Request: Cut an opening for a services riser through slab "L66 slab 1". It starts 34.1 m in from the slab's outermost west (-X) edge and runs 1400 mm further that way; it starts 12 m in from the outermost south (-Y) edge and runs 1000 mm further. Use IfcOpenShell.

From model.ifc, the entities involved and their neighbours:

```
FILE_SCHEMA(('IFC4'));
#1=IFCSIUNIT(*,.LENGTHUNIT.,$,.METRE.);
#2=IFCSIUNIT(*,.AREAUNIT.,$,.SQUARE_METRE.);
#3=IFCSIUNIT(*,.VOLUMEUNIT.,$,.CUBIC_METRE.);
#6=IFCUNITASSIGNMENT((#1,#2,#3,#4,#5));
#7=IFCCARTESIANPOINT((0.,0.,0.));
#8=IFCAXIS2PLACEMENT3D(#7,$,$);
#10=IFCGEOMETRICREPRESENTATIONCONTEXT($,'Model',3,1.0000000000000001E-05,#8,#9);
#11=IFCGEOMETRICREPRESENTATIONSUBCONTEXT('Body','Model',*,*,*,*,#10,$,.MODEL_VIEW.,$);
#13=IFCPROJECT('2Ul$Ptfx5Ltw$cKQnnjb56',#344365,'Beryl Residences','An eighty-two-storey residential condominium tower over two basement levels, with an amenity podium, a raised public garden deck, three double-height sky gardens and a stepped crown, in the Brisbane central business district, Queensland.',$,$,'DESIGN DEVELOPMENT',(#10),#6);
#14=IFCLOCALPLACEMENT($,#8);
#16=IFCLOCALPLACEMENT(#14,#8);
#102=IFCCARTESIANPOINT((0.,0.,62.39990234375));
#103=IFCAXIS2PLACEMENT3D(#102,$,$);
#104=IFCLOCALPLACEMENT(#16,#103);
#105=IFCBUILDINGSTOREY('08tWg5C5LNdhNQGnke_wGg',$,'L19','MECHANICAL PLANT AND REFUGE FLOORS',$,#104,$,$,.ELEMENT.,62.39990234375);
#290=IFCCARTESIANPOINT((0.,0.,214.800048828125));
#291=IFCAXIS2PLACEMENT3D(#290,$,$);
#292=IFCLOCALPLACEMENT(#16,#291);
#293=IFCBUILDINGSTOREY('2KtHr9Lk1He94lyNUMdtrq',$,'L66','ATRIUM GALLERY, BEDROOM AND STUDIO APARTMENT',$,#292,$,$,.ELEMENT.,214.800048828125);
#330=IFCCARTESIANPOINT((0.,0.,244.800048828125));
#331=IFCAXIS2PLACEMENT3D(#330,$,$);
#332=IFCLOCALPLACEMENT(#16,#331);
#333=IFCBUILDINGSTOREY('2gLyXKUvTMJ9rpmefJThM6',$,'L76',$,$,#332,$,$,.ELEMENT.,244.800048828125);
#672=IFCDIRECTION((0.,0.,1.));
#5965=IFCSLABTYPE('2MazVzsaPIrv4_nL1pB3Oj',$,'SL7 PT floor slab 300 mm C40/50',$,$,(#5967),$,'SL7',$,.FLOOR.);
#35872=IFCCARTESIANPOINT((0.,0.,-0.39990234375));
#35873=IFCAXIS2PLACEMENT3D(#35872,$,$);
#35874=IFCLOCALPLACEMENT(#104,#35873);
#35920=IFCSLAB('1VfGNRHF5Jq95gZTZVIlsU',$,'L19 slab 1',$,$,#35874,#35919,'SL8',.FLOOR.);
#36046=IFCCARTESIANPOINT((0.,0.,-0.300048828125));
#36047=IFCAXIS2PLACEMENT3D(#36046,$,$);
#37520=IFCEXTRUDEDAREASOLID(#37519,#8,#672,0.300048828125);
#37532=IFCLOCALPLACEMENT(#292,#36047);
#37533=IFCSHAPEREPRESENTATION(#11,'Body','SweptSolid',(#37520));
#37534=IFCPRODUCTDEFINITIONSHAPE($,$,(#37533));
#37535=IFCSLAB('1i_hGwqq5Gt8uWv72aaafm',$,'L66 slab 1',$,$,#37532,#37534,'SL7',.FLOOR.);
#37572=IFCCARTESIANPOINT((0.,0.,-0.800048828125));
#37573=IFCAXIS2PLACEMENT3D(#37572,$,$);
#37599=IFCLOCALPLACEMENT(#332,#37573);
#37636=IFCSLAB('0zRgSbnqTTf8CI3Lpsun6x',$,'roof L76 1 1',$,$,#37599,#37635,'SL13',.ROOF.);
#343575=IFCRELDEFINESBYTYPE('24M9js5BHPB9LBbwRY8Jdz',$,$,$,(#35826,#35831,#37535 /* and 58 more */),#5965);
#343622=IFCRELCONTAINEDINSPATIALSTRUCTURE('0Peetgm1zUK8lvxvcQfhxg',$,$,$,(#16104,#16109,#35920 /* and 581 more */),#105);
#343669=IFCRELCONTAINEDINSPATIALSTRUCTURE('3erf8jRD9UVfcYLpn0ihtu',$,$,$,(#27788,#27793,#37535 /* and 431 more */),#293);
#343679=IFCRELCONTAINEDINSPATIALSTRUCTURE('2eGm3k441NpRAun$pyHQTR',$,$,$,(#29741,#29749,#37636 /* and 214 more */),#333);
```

```python
import numpy as np
import ifcopenshell
import ifcopenshell.api.feature
import ifcopenshell.api.geometry
import ifcopenshell.api.root
import ifcopenshell.geom
import ifcopenshell.util.placement
import ifcopenshell.util.representation
import ifcopenshell.util.shape
import ifcopenshell.util.unit

model = ifcopenshell.open("model.ifc")
unit_scale = ifcopenshell.util.unit.calculate_unit_scale(model)
settings = ifcopenshell.geom.settings()


def volume(element):
    """Net volume in cubic metres, openings subtracted."""
    shape = ifcopenshell.geom.create_shape(settings, element)
    return ifcopenshell.util.shape.get_volume(shape.geometry)


slab = model.by_guid("1i_hGwqq5Gt8uWv72aaafm")
before = volume(slab)

# Extent in the slab's own axes, in metres. The edges named are its -X and -Y sides.
slab_shape = ifcopenshell.geom.create_shape(settings, slab)
vertices = ifcopenshell.util.shape.get_vertices(slab_shape.geometry)
x_min, y_min, bottom = vertices.min(axis=0)
top = vertices[:, 2].max()

opening = ifcopenshell.api.root.create_entity(model, ifc_class="IfcOpeningElement", name="Services riser opening", predefined_type="OPENING")
context = ifcopenshell.util.representation.get_context(model, "Model", "Body", "MODEL_VIEW")
width, depth = 1.4, 1
outline = [(0.0, 0.0), (width, 0.0), (width, depth), (0.0, depth), (0.0, 0.0)]
# Overshoot both faces by 50 mm so the cut is clean.
shape = ifcopenshell.api.geometry.add_slab_representation(
    model, context=context, depth=top - bottom + 0.1, polyline=outline
)
ifcopenshell.api.geometry.assign_representation(model, product=opening, representation=shape)

matrix = ifcopenshell.util.placement.get_local_placement(slab.ObjectPlacement)
matrix[:, 3] = matrix @ np.append(np.array([x_min + 34.1, y_min + 12, bottom - 0.05]) / unit_scale, 1.0)
ifcopenshell.api.geometry.edit_object_placement(model, product=opening, matrix=matrix, is_si=False)
ifcopenshell.api.feature.add_feature(model, feature=opening, element=slab)

after = volume(slab)

print(f"slab volume {before:.3f} -> {after:.3f} m3")

model.write("model_edited.ifc")
```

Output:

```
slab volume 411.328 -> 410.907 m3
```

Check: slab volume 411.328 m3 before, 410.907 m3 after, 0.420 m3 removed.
